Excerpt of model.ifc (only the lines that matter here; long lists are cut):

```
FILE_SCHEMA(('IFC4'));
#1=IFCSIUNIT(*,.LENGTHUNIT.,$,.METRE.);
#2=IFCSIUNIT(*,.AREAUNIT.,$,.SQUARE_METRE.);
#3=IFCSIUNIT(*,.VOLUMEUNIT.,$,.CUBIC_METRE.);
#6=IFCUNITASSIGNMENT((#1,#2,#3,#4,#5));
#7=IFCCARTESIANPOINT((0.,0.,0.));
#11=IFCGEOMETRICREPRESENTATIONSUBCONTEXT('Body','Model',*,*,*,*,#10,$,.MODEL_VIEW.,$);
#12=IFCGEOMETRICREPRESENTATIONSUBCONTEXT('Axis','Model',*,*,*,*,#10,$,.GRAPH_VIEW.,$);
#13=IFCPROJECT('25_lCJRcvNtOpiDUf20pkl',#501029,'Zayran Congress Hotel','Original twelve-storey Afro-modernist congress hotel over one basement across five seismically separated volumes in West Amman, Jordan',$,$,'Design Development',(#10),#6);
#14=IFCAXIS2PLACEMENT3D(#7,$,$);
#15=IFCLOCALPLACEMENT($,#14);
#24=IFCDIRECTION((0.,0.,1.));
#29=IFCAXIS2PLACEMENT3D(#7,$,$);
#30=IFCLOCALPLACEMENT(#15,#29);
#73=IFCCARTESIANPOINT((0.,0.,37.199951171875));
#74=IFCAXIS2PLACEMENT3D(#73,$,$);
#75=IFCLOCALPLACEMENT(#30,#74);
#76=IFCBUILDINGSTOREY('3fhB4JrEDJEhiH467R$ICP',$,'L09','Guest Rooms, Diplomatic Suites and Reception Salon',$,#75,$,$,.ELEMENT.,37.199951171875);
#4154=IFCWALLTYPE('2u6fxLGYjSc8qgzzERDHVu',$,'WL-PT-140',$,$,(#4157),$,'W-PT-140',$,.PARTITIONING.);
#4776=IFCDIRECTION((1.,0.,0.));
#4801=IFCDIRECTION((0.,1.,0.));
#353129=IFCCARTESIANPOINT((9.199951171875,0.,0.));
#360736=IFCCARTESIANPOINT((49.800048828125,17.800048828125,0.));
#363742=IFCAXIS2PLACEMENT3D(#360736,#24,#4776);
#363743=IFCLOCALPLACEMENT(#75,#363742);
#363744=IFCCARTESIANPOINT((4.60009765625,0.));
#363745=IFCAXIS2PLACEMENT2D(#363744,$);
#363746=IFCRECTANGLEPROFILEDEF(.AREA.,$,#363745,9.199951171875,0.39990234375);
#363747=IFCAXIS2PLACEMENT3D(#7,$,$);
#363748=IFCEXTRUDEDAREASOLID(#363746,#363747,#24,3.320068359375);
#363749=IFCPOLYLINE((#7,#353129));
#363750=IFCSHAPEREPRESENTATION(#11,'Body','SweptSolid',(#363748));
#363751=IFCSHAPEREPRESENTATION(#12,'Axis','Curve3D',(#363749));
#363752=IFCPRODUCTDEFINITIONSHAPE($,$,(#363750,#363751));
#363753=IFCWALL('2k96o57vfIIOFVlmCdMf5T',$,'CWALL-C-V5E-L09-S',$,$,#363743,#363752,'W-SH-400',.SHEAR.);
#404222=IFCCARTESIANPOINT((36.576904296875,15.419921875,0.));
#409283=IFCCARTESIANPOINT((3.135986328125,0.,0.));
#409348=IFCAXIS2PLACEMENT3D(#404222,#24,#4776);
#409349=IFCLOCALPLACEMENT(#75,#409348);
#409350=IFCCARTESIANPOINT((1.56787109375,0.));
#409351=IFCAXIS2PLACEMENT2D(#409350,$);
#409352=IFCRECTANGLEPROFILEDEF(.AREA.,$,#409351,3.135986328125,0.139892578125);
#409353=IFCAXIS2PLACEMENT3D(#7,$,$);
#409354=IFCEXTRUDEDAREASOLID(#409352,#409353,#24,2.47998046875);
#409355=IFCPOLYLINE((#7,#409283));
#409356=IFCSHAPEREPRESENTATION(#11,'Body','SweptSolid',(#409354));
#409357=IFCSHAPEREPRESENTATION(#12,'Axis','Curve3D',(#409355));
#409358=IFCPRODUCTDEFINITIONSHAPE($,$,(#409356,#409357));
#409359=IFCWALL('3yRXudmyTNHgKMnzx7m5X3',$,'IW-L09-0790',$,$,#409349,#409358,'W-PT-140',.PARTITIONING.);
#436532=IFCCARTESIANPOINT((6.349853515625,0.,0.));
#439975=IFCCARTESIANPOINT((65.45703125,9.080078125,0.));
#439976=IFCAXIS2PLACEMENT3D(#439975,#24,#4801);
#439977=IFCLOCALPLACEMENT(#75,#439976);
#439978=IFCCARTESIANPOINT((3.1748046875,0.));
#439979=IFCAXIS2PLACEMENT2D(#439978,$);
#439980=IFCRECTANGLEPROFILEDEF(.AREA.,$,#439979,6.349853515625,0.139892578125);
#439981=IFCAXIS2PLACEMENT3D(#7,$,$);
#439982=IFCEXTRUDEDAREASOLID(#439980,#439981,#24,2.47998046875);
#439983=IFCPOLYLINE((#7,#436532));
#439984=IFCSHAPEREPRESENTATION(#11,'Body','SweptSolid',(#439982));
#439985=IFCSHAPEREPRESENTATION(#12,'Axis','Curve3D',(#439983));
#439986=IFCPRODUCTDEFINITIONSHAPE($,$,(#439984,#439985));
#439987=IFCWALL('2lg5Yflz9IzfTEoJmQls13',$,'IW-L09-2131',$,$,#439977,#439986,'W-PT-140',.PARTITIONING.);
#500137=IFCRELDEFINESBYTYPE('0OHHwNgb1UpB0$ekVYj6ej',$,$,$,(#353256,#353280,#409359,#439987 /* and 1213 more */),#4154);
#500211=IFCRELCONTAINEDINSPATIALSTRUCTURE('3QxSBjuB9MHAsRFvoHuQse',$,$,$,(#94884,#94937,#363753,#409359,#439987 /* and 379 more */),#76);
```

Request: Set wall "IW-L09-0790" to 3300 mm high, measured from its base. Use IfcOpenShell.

```python
import ifcopenshell
import ifcopenshell.geom
import ifcopenshell.util.representation
import ifcopenshell.util.shape
import ifcopenshell.util.unit

model = ifcopenshell.open("model.ifc")
unit_scale = ifcopenshell.util.unit.calculate_unit_scale(model)
settings = ifcopenshell.geom.settings()


def volume(element):
    """Net volume in cubic metres, openings subtracted."""
    shape = ifcopenshell.geom.create_shape(settings, element)
    return ifcopenshell.util.shape.get_volume(shape.geometry)


wall = model.by_guid("3yRXudmyTNHgKMnzx7m5X3")
before = volume(wall)

body = ifcopenshell.util.representation.get_representation(wall, "Model", "Body")
solid = body.Items[0]
old_height = solid.Depth
solid.Depth = 3.3 / unit_scale
after = volume(wall)

print(f"height {old_height:g} -> {solid.Depth:g}, volume {before:.3f} -> {after:.3f} m3")

model.write("model_v2.ifc")
```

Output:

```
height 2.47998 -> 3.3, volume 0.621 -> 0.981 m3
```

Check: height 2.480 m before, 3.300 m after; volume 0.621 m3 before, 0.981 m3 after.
